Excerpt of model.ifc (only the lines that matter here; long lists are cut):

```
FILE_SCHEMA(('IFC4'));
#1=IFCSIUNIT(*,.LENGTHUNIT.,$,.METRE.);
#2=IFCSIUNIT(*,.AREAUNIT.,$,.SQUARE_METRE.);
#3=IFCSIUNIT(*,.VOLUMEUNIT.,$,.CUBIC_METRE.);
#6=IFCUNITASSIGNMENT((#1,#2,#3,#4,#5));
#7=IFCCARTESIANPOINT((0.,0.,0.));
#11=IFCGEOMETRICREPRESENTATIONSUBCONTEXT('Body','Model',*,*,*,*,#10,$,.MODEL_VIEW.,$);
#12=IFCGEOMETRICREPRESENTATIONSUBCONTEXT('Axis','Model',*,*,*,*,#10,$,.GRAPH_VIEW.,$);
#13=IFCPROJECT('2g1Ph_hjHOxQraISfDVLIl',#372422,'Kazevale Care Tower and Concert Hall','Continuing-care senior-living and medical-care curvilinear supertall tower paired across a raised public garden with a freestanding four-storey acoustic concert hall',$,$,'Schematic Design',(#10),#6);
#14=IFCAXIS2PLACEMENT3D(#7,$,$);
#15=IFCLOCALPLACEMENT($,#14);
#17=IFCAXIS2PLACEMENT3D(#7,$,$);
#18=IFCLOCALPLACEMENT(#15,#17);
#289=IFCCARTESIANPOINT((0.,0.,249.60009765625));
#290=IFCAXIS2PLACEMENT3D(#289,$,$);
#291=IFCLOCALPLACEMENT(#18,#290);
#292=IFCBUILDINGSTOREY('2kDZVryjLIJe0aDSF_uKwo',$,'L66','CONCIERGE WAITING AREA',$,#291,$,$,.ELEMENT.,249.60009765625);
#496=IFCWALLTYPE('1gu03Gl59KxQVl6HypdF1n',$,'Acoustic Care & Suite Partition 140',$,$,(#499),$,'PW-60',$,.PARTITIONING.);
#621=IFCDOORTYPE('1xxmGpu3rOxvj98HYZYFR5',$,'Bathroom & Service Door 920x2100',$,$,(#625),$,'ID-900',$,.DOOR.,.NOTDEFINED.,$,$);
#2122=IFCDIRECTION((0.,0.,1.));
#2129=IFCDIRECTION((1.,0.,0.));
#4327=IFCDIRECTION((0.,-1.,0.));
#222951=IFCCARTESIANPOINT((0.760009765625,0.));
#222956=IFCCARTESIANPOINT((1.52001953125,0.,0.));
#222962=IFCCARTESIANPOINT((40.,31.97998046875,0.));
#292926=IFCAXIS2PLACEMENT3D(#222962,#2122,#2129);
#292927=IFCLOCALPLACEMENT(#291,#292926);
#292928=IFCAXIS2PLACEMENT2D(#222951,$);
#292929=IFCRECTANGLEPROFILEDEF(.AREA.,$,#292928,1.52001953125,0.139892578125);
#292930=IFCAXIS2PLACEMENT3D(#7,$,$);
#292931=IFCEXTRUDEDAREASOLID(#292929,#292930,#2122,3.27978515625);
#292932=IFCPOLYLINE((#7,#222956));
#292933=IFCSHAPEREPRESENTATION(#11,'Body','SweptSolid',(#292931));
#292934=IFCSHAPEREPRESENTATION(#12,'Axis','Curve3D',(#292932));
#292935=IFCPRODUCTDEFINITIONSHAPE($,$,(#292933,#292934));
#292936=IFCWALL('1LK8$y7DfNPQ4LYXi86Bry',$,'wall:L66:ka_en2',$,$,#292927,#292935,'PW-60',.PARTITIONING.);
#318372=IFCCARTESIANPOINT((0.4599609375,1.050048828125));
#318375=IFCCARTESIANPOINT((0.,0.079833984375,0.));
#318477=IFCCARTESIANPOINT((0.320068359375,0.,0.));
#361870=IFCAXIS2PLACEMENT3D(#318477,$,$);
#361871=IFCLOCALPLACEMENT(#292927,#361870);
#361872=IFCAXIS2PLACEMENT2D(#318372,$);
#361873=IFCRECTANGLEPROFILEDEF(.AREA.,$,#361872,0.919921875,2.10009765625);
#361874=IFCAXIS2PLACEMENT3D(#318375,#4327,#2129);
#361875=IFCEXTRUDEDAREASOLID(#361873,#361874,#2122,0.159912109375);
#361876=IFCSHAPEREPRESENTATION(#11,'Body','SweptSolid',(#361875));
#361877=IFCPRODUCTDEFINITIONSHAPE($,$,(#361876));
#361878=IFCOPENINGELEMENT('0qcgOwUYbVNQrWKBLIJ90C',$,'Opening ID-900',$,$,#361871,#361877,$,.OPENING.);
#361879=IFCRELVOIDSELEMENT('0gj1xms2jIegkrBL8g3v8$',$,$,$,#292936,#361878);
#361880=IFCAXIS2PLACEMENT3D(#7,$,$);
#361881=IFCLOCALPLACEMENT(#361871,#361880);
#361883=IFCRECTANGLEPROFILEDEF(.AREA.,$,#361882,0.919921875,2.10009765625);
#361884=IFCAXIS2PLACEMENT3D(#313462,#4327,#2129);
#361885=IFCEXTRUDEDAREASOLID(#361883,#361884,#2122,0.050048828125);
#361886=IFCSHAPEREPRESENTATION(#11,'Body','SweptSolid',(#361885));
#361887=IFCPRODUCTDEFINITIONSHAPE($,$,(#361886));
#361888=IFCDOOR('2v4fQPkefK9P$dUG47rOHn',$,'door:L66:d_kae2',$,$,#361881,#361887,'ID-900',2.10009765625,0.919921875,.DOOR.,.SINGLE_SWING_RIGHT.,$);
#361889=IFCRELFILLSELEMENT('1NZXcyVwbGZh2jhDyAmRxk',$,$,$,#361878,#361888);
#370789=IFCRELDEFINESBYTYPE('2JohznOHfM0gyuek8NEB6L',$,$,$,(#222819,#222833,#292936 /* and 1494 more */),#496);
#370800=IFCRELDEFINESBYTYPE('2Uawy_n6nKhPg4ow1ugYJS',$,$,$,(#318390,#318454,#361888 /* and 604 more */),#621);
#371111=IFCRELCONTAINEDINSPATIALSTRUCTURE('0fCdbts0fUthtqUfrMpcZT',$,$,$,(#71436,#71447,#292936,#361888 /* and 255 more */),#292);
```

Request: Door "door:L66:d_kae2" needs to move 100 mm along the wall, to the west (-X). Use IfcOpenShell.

```python
import ifcopenshell
import ifcopenshell.api.geometry
import ifcopenshell.util.placement

model = ifcopenshell.open("model.ifc")

door = model.by_guid("2v4fQPkefK9P$dUG47rOHn")
opening = door.FillsVoids[0].RelatingOpeningElement
wall = opening.VoidsElements[0].RelatingBuildingElement

wall_matrix = ifcopenshell.util.placement.get_local_placement(wall.ObjectPlacement)
shift = wall_matrix[:3, 0] * -0.1
before = ifcopenshell.util.placement.get_local_placement(door.ObjectPlacement)[:3, 3].copy()

# The door is placed relative to its opening, so it follows when the opening moves.
matrix = ifcopenshell.util.placement.get_local_placement(opening.ObjectPlacement)
matrix[:3, 3] += shift
ifcopenshell.api.geometry.edit_object_placement(
    model, product=opening, matrix=matrix, is_si=False, should_transform_children=True
)

after = ifcopenshell.util.placement.get_local_placement(door.ObjectPlacement)[:3, 3]
print("door moved by", (after - before).round(3) + 0.0)

model.write("model-out.ifc")
```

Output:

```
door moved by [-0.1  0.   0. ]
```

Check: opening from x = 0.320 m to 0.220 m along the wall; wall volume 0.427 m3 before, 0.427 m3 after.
